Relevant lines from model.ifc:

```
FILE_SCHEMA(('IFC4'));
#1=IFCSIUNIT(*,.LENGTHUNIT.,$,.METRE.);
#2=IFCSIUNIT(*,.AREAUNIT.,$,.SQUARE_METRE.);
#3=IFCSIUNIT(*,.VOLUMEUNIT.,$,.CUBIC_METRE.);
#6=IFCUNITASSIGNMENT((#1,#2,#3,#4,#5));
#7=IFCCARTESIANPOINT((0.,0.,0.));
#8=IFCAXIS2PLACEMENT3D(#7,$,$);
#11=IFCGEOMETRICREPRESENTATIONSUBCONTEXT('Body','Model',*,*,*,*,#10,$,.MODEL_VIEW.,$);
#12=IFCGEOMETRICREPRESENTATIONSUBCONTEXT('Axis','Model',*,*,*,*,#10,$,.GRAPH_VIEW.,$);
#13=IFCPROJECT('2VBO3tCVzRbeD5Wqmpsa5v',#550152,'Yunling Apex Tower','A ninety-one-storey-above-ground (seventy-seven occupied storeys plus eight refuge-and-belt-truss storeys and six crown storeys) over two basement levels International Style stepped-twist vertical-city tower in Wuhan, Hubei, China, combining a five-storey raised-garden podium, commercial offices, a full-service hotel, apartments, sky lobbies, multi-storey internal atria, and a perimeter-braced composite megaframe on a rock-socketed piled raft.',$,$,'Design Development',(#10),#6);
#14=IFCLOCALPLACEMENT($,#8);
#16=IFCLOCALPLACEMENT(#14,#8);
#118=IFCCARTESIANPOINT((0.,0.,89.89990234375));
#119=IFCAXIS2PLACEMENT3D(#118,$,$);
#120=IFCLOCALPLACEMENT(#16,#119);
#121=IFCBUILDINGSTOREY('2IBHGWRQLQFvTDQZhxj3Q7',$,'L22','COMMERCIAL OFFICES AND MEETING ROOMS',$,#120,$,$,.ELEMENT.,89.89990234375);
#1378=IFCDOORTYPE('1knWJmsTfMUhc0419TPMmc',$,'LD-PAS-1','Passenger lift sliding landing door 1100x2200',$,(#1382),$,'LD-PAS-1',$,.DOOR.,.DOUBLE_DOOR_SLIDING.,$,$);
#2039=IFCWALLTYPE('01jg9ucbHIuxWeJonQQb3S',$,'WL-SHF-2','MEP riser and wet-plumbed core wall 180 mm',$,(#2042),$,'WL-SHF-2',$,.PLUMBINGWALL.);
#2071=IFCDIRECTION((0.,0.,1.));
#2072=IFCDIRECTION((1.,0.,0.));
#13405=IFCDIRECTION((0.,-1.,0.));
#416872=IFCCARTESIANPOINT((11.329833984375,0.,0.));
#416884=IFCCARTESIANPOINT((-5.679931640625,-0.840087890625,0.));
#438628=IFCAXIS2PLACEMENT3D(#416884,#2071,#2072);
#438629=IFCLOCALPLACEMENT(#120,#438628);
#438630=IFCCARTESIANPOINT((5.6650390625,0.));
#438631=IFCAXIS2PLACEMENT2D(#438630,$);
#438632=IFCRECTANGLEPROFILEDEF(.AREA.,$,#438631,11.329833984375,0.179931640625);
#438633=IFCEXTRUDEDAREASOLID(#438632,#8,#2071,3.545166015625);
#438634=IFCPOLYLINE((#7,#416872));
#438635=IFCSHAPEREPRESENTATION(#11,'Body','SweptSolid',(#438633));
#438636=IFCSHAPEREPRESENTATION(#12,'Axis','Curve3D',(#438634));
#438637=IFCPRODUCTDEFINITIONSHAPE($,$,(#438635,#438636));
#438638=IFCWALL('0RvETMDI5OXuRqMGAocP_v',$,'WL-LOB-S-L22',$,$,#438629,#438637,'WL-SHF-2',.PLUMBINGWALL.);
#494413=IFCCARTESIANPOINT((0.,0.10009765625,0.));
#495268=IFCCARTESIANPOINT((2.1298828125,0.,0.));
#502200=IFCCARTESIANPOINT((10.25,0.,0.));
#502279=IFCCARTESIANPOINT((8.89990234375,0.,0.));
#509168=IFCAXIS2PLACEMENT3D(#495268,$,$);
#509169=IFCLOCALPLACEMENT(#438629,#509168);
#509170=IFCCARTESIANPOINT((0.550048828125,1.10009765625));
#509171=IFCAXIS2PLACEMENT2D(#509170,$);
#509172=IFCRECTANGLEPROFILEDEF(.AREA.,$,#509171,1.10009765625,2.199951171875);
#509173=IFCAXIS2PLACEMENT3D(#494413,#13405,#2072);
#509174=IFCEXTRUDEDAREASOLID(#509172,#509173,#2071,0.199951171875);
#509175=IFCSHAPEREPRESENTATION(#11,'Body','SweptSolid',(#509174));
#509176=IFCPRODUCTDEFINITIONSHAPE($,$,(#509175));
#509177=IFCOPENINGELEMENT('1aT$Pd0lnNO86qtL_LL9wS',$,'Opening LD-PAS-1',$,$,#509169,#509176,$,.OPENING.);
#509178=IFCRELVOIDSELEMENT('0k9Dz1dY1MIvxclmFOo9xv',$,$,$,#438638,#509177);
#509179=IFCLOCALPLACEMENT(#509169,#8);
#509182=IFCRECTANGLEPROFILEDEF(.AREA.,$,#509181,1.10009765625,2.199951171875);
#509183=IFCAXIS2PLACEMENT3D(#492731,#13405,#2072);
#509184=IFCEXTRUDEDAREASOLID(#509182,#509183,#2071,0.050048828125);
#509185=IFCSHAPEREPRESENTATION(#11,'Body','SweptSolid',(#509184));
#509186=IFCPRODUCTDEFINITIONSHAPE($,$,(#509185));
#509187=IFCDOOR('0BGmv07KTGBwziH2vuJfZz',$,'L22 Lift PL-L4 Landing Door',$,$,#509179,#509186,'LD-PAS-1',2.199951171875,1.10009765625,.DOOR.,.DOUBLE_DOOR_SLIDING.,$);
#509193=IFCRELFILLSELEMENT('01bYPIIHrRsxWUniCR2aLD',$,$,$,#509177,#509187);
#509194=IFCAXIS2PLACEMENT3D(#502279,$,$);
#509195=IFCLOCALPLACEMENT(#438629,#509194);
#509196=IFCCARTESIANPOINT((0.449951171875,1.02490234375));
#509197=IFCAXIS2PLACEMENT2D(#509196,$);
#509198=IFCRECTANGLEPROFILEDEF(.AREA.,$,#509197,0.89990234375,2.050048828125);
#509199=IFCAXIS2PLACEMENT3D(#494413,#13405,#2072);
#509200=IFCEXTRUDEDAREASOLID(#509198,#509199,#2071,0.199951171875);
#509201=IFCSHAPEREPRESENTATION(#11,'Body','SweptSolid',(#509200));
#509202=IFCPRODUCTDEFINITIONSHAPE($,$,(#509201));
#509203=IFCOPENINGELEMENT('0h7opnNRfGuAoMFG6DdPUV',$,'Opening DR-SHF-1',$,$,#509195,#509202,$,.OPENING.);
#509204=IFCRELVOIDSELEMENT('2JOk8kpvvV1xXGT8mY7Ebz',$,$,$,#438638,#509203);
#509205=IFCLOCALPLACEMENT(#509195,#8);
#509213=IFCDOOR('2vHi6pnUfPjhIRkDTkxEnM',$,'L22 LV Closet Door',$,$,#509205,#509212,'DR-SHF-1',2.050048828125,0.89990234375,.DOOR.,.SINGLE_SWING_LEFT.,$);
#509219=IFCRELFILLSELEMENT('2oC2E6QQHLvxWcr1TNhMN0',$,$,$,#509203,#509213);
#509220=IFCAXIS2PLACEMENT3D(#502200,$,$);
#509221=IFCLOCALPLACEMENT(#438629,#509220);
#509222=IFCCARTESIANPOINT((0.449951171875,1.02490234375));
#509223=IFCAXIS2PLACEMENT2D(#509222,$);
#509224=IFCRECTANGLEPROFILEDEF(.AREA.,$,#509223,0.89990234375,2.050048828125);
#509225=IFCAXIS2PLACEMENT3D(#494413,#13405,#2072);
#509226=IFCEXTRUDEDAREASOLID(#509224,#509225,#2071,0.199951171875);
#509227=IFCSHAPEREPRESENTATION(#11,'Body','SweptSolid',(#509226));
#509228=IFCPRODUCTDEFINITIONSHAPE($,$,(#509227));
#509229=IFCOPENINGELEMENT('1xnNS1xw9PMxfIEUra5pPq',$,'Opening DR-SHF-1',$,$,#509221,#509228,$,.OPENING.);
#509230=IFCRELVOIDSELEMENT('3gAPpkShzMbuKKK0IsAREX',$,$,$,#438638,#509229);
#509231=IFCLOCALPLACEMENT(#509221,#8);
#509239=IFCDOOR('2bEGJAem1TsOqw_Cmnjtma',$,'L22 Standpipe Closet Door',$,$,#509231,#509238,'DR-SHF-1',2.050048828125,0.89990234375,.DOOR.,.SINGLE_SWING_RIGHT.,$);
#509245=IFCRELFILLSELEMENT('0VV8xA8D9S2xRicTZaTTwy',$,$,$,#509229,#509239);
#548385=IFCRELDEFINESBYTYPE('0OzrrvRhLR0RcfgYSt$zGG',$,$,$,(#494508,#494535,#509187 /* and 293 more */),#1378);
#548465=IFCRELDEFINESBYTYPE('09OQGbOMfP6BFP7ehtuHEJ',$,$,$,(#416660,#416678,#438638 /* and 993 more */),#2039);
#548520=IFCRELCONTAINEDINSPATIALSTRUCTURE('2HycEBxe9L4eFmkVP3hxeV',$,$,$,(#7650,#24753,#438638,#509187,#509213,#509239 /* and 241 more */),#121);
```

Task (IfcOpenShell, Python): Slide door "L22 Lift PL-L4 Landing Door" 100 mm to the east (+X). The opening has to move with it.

```python
import ifcopenshell
import ifcopenshell.api.geometry
import ifcopenshell.util.placement
import ifcopenshell.util.unit

model = ifcopenshell.open("model.ifc")
unit_scale = ifcopenshell.util.unit.calculate_unit_scale(model)

door = model.by_id(509187)
opening = door.FillsVoids[0].RelatingOpeningElement
wall = opening.VoidsElements[0].RelatingBuildingElement

wall_matrix = ifcopenshell.util.placement.get_local_placement(wall.ObjectPlacement)
shift = wall_matrix[:3, 0] * 0.1 / unit_scale
before = ifcopenshell.util.placement.get_local_placement(door.ObjectPlacement)[:3, 3].copy()

# The door is placed relative to its opening, so it follows when the opening moves.
matrix = ifcopenshell.util.placement.get_local_placement(opening.ObjectPlacement)
matrix[:3, 3] += shift
ifcopenshell.api.geometry.edit_object_placement(
    model, product=opening, matrix=matrix, is_si=False, should_transform_children=True
)

after = ifcopenshell.util.placement.get_local_placement(door.ObjectPlacement)[:3, 3]
print("door moved by", (after - before).round(3) + 0.0)

model.write("model_edited.ifc")
```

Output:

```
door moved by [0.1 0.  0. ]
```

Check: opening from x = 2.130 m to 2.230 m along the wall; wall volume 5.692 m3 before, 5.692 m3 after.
